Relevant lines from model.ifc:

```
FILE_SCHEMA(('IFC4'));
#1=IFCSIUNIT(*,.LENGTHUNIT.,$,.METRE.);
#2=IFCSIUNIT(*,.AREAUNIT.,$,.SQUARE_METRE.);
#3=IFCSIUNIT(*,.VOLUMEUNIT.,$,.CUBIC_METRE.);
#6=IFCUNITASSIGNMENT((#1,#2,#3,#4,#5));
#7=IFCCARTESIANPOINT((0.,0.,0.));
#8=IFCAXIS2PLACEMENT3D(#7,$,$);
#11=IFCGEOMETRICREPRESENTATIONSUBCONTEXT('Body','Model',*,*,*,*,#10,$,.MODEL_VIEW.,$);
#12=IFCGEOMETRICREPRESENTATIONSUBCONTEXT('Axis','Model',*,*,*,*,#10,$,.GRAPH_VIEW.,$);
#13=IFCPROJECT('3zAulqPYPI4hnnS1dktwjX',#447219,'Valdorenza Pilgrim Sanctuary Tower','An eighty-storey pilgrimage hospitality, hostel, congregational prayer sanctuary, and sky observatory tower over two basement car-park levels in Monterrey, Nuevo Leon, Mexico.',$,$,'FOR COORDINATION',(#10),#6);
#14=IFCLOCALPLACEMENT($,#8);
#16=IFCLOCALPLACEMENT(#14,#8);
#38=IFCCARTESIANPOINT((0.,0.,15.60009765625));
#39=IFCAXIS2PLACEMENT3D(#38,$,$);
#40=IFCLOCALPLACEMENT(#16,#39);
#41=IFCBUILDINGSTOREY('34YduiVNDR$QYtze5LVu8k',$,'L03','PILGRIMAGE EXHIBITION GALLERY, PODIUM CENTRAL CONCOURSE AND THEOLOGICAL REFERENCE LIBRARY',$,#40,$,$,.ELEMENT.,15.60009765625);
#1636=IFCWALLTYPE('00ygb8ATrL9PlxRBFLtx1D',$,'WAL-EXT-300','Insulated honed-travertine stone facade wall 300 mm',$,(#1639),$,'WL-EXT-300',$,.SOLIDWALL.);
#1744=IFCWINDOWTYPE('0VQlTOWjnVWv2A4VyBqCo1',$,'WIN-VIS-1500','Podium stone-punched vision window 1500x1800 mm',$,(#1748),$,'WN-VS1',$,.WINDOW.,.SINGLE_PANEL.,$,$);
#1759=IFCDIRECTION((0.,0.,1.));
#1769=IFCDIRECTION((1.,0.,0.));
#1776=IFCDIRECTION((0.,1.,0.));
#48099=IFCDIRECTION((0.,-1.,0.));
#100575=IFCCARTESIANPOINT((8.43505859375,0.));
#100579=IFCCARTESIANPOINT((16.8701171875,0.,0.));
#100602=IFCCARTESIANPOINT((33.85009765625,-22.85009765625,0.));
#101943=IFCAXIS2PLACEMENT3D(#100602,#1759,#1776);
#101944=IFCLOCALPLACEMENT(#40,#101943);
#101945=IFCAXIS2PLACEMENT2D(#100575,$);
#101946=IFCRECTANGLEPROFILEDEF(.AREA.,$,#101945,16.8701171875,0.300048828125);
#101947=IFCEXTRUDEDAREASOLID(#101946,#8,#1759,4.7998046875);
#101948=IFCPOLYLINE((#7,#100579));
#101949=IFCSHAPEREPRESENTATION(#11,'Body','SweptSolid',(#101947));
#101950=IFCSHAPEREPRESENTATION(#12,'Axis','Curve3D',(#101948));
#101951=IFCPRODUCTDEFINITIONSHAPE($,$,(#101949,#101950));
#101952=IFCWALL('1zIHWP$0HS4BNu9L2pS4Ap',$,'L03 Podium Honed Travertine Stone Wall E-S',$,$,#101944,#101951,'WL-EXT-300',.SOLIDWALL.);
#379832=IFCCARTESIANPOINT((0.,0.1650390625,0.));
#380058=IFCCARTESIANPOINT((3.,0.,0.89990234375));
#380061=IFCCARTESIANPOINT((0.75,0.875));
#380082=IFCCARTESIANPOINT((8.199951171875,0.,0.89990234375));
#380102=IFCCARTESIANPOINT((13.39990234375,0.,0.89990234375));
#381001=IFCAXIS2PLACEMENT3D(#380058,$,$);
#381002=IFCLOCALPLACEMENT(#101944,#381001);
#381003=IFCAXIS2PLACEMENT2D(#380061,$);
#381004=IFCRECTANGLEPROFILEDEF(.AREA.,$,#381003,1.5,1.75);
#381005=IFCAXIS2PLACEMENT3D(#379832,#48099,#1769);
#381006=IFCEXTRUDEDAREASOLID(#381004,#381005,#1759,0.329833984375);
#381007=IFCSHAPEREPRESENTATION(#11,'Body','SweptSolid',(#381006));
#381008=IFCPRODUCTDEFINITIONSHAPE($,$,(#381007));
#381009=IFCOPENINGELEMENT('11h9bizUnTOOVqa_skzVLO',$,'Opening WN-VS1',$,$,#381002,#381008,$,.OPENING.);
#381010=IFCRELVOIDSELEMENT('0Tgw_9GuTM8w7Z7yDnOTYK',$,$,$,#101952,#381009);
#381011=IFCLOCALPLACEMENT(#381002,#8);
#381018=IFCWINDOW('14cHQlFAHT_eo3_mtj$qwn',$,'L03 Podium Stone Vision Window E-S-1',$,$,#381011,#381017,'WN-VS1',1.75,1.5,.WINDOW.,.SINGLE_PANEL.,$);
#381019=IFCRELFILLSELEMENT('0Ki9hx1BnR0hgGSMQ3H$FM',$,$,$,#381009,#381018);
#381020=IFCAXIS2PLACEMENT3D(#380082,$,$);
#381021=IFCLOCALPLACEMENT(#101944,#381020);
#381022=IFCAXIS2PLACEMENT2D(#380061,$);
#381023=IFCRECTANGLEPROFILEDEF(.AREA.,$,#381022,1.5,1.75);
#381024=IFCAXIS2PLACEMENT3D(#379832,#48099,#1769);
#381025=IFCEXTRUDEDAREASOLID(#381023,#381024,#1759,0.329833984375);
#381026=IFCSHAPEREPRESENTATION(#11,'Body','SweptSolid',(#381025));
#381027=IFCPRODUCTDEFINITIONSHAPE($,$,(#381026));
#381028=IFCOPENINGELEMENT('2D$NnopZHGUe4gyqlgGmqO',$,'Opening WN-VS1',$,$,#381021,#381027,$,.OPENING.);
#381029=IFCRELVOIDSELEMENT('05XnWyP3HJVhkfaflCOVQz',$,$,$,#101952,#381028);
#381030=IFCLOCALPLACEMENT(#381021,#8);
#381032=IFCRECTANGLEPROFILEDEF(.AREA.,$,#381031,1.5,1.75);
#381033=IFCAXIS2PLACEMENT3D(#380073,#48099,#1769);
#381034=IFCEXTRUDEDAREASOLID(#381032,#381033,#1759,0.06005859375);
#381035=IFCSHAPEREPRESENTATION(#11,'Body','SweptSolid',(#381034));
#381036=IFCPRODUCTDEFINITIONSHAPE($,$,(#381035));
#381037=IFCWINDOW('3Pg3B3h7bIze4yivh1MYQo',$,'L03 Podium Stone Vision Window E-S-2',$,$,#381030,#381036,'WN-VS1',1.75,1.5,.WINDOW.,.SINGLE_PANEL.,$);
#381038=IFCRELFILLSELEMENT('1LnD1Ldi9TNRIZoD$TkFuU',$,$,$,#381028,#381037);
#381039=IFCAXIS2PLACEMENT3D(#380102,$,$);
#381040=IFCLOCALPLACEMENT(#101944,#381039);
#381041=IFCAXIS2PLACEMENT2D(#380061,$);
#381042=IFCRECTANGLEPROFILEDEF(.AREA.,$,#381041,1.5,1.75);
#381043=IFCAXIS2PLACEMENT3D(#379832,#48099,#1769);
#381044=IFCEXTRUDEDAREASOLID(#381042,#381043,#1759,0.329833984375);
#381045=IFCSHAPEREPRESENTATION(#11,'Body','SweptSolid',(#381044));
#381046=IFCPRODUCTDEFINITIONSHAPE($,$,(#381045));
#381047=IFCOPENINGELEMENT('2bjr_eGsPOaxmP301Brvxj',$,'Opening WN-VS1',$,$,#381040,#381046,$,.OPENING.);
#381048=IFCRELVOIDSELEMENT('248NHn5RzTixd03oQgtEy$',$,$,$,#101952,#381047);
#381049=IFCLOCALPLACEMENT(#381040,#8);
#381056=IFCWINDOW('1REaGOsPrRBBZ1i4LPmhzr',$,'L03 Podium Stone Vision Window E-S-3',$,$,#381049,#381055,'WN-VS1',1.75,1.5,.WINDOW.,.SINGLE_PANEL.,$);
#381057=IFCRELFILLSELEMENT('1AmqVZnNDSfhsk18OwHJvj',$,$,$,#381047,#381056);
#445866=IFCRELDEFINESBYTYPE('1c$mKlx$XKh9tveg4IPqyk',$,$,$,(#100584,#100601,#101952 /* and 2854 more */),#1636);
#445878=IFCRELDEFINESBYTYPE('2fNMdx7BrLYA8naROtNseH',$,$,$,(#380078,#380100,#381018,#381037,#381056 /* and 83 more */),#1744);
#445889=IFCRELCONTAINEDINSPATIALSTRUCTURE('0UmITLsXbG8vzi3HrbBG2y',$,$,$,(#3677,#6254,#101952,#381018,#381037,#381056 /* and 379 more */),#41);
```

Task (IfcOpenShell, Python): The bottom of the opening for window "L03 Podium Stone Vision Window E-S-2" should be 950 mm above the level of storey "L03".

```python
import numpy as np
import ifcopenshell
import ifcopenshell.api.geometry
import ifcopenshell.geom
import ifcopenshell.util.element
import ifcopenshell.util.placement
import ifcopenshell.util.shape
import ifcopenshell.util.unit

model = ifcopenshell.open("model.ifc")
unit_scale = ifcopenshell.util.unit.calculate_unit_scale(model)

window = model.by_id(381037)
opening = window.FillsVoids[0].RelatingOpeningElement
storey = ifcopenshell.util.element.get_container(window, ifc_class="IfcBuildingStorey")
level = ifcopenshell.util.placement.get_local_placement(storey.ObjectPlacement)[2, 3]

# The opening's origin need not be at the sill, so measure its lowest point.
shape = ifcopenshell.geom.create_shape(ifcopenshell.geom.settings(), opening)
bottom = ifcopenshell.util.shape.get_shape_bottom_elevation(shape, shape.geometry) / unit_scale
dz = level + 0.95 / unit_scale - bottom

shift = np.array([0.0, 0.0, dz])
# The window is placed relative to its opening, so it follows when the opening moves.
matrix = ifcopenshell.util.placement.get_local_placement(opening.ObjectPlacement)
matrix[:3, 3] += shift
ifcopenshell.api.geometry.edit_object_placement(
    model, product=opening, matrix=matrix, is_si=False, should_transform_children=True
)

print(f"moved by {dz * unit_scale:+.3f} m")

model.write("model_v2.ifc")
```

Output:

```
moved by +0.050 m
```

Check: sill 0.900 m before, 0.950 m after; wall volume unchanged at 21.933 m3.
